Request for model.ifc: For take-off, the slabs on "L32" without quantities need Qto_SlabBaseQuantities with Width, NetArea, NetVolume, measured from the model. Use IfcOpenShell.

First a look at what the model holds.

```python
import ifcopenshell
import ifcopenshell.util.element
import ifcopenshell.util.unit

model = ifcopenshell.open("model.ifc")
print(model.schema)
for unit_type in ("LENGTHUNIT", "AREAUNIT", "VOLUMEUNIT"):
    print(unit_type, ifcopenshell.util.unit.calculate_unit_scale(model, unit_type))
storey = next(s for s in model.by_type("IfcBuildingStorey") if s.Name == "L32")
slabs = [e for e in ifcopenshell.util.element.get_decomposition(storey) if e.is_a("IfcSlab")]
for e in sorted(slabs, key=lambda e: e.id()):
    print(e.id(), e.is_a(), e.Name, list(ifcopenshell.util.element.get_psets(e, qtos_only=True)), sep=" | ")
```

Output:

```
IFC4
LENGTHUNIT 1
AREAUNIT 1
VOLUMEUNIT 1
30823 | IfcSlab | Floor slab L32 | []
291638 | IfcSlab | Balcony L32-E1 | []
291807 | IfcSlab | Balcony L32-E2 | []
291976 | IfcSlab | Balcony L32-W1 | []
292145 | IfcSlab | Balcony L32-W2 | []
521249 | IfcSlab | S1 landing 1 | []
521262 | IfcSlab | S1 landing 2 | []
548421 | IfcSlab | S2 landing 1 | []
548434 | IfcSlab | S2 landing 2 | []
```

```python
import ifcopenshell
import ifcopenshell.api.pset
import ifcopenshell.geom
import ifcopenshell.util.element
import ifcopenshell.util.shape
import ifcopenshell.util.unit

model = ifcopenshell.open("model.ifc")
unit_scale = ifcopenshell.util.unit.calculate_unit_scale(model)
area_scale = ifcopenshell.util.unit.calculate_unit_scale(model, "AREAUNIT")
volume_scale = ifcopenshell.util.unit.calculate_unit_scale(model, "VOLUMEUNIT")
settings = ifcopenshell.geom.settings()

storey = next(s for s in model.by_type("IfcBuildingStorey") if s.Name == "L32")
slabs = [e for e in ifcopenshell.util.element.get_decomposition(storey) if e.is_a("IfcSlab")]

for e in sorted(slabs, key=lambda e: e.id()):
    if ifcopenshell.util.element.get_psets(e, qtos_only=True, should_inherit=False):
        continue
    # Geometry comes back in metres, in the element's own axes.
    shape = ifcopenshell.geom.create_shape(settings, e)
    values = {
        "Width": ifcopenshell.util.shape.get_z(shape.geometry) / unit_scale,
        "NetArea": ifcopenshell.util.shape.get_footprint_area(shape.geometry) / area_scale,
        "NetVolume": ifcopenshell.util.shape.get_volume(shape.geometry) / volume_scale,
    }
    qto = ifcopenshell.api.pset.add_qto(model, product=e, name="Qto_SlabBaseQuantities")
    ifcopenshell.api.pset.edit_qto(model, qto=qto, properties=values)
    print(e.id(), {k: round(v, 3) for k, v in values.items()})

model.write("model_rev.ifc")
```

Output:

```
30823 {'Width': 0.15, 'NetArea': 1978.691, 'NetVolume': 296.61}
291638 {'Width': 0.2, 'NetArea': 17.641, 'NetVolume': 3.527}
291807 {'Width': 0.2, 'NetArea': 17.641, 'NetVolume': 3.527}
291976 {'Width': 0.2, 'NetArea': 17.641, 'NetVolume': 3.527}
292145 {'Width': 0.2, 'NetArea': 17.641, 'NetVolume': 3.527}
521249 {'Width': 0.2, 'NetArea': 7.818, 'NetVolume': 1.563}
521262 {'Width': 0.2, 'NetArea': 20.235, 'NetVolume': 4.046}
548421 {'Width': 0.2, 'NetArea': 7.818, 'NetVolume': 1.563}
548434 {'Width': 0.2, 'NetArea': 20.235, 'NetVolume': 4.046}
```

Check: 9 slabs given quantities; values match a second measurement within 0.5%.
